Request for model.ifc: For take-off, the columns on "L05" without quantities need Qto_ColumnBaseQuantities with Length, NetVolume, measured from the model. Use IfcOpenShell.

First a look at what the model holds.

```python
import ifcopenshell
import ifcopenshell.util.element
import ifcopenshell.util.unit

model = ifcopenshell.open("model.ifc")
print(model.schema)
for unit_type in ("LENGTHUNIT", "AREAUNIT", "VOLUMEUNIT"):
    print(unit_type, ifcopenshell.util.unit.calculate_unit_scale(model, unit_type))
storey = next(s for s in model.by_type("IfcBuildingStorey") if s.Name == "L05")
columns = [e for e in ifcopenshell.util.element.get_decomposition(storey) if e.is_a("IfcColumn")]
for e in sorted(columns, key=lambda e: e.id()):
    print(e.id(), e.is_a(), e.Name, list(ifcopenshell.util.element.get_psets(e, qtos_only=True)), sep=" | ")
```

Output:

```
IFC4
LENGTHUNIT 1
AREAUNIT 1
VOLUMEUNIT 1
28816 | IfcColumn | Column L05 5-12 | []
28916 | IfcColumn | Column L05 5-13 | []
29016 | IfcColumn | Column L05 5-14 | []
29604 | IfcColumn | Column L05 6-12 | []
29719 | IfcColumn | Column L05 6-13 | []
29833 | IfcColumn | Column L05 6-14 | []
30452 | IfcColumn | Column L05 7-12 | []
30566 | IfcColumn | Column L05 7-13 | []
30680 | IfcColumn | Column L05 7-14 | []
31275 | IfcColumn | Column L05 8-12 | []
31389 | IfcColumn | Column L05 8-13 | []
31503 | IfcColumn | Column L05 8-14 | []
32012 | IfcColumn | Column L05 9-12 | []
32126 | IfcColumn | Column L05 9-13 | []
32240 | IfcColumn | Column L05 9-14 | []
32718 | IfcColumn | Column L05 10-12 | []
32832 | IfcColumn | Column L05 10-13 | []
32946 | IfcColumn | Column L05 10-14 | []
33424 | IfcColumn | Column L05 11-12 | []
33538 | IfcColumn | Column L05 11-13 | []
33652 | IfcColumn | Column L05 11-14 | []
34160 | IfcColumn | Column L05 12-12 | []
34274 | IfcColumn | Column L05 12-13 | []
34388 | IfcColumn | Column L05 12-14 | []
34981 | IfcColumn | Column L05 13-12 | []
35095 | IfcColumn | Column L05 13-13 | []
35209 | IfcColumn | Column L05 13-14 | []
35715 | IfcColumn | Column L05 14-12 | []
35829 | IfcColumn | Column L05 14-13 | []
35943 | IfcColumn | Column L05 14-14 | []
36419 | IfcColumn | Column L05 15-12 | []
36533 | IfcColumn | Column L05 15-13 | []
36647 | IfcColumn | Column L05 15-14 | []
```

```python
import ifcopenshell
import ifcopenshell.api.pset
import ifcopenshell.geom
import ifcopenshell.util.element
import ifcopenshell.util.shape
import ifcopenshell.util.unit

model = ifcopenshell.open("model.ifc")
unit_scale = ifcopenshell.util.unit.calculate_unit_scale(model)
volume_scale = ifcopenshell.util.unit.calculate_unit_scale(model, "VOLUMEUNIT")
settings = ifcopenshell.geom.settings()

storey = next(s for s in model.by_type("IfcBuildingStorey") if s.Name == "L05")
columns = [e for e in ifcopenshell.util.element.get_decomposition(storey) if e.is_a("IfcColumn")]

for e in sorted(columns, key=lambda e: e.id()):
    if ifcopenshell.util.element.get_psets(e, qtos_only=True, should_inherit=False):
        continue
    # Geometry comes back in metres, in the element's own axes.
    shape = ifcopenshell.geom.create_shape(settings, e)
    values = {
        "Length": ifcopenshell.util.shape.get_z(shape.geometry) / unit_scale,
        "NetVolume": ifcopenshell.util.shape.get_volume(shape.geometry) / volume_scale,
    }
    qto = ifcopenshell.api.pset.add_qto(model, product=e, name="Qto_ColumnBaseQuantities")
    ifcopenshell.api.pset.edit_qto(model, qto=qto, properties=values)
    print(e.id(), {k: round(v, 3) for k, v in values.items()})

model.write("model_v2.ifc")
```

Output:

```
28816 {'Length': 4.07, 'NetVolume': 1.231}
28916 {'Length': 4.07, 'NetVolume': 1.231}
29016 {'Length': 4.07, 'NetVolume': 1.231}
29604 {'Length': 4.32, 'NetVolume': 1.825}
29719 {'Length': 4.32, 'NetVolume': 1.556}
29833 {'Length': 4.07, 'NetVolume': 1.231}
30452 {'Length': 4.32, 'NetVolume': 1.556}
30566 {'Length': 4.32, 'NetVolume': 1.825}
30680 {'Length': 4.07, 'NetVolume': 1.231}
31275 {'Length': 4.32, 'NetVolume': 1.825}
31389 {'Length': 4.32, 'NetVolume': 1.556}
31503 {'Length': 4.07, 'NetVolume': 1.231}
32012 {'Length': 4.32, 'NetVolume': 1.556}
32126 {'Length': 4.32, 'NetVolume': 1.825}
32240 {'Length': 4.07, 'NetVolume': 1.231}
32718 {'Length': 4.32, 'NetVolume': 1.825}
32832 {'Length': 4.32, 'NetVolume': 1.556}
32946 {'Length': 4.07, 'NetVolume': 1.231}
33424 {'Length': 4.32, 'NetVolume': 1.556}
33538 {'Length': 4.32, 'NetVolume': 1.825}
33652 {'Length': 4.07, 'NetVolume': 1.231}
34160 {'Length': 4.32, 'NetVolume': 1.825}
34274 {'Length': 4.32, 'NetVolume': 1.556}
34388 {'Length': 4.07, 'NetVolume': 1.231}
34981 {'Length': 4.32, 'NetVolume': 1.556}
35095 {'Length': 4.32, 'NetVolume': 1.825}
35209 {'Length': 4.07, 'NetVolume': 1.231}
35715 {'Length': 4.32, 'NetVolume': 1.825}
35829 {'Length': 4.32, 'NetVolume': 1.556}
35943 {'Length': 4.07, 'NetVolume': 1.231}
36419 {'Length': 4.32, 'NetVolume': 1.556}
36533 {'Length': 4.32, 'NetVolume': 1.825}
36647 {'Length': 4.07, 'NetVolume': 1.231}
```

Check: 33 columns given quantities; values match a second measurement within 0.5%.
